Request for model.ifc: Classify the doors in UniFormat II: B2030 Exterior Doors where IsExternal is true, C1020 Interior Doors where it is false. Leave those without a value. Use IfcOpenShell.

First a look at what the model holds.

```python
import ifcopenshell
import ifcopenshell.util.element

model = ifcopenshell.open("model.ifc")
print(model.schema)
print("classifications:", [c.Name for c in model.by_type("IfcClassification")])
values = [ifcopenshell.util.element.get_pset(e, "Pset_DoorCommon", "IsExternal") for e in model.by_type("IfcDoor")]
for value in (True, False, None):
    print("IsExternal", value, values.count(value))
```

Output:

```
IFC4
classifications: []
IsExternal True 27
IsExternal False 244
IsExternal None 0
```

```python
import ifcopenshell
import ifcopenshell.api.classification
import ifcopenshell.util.element

model = ifcopenshell.open("model.ifc")

system = ifcopenshell.api.classification.add_classification(model, classification="UniFormat II")

doors = model.by_type("IfcDoor")
external = {e: ifcopenshell.util.element.get_pset(e, "Pset_DoorCommon", "IsExternal") for e in doors}
for flag, code, name in ((True, "B2030", "Exterior Doors"), (False, "C1020", "Interior Doors")):
    products = [e for e in doors if external[e] is flag]
    ifcopenshell.api.classification.add_reference(
        model, products=products, classification=system, identification=code, name=name
    )
    print(code, len(products))

model.write("model_updated.ifc")
```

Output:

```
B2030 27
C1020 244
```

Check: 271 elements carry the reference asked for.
